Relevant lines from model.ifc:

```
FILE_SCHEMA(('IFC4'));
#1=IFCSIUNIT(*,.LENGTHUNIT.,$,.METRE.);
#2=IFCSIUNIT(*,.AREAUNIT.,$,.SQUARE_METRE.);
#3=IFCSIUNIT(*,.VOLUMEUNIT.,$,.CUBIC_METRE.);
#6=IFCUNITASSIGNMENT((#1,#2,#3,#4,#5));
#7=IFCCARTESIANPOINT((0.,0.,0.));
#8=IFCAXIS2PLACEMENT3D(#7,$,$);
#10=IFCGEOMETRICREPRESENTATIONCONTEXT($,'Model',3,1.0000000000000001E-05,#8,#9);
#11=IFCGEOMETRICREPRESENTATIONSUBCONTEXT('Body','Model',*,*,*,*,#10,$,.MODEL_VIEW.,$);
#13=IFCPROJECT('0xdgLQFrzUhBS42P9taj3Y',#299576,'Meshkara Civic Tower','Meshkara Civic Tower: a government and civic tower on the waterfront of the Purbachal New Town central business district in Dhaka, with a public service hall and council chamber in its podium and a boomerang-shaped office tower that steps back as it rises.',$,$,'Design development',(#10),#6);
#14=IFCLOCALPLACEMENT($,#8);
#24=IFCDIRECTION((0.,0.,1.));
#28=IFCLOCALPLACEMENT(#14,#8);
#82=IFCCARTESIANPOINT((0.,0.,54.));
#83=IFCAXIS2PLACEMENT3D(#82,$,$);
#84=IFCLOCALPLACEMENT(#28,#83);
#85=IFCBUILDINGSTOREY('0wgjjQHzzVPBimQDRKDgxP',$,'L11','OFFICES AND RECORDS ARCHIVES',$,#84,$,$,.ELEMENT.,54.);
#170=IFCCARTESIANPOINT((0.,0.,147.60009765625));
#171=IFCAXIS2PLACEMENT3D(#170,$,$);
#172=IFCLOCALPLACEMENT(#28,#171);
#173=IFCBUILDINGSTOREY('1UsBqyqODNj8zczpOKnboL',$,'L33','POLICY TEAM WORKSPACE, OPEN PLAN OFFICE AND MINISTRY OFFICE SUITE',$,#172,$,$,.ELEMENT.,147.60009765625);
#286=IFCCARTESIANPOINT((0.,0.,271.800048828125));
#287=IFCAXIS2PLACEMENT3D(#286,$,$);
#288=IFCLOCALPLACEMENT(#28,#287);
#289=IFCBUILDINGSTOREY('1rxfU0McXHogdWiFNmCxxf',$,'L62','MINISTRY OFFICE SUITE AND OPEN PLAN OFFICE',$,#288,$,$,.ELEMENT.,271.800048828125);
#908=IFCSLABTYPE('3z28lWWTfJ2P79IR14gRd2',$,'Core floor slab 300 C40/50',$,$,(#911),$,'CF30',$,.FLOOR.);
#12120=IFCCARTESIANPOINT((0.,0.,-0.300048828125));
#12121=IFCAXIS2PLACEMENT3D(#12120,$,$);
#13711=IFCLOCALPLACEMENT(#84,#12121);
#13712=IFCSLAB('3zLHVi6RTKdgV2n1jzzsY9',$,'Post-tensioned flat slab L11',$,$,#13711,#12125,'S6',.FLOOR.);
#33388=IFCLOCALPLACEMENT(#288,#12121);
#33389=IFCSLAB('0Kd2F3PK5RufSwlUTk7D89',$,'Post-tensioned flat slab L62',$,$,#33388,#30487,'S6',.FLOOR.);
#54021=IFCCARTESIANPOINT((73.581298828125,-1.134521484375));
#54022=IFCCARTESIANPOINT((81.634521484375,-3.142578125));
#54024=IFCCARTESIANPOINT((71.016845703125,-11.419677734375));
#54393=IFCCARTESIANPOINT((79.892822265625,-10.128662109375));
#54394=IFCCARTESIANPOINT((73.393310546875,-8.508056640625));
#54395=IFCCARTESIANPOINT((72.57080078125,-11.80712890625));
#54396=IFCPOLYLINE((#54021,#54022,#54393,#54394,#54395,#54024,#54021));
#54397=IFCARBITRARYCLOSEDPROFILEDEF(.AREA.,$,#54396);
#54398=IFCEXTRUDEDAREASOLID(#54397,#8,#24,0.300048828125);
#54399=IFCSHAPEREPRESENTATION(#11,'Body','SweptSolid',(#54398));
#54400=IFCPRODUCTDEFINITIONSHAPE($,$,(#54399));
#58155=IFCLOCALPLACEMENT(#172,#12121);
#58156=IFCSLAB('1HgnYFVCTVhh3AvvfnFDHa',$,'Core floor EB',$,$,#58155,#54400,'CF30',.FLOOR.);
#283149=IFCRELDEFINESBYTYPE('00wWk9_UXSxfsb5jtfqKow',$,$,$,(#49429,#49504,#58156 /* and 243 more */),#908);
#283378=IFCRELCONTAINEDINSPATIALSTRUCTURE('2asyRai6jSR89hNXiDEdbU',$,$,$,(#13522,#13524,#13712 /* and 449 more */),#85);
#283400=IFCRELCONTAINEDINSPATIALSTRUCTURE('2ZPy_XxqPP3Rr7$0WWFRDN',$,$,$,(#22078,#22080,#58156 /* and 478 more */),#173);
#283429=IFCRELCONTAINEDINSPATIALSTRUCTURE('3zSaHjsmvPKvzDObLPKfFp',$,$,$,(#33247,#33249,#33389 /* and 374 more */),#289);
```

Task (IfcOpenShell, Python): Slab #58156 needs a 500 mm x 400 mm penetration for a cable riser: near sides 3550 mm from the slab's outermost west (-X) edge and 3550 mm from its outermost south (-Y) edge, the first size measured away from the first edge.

```python
import numpy as np
import ifcopenshell
import ifcopenshell.api.feature
import ifcopenshell.api.geometry
import ifcopenshell.api.root
import ifcopenshell.geom
import ifcopenshell.util.placement
import ifcopenshell.util.representation
import ifcopenshell.util.shape
import ifcopenshell.util.unit

model = ifcopenshell.open("model.ifc")
unit_scale = ifcopenshell.util.unit.calculate_unit_scale(model)
settings = ifcopenshell.geom.settings()


def volume(element):
    """Net volume in cubic metres, openings subtracted."""
    shape = ifcopenshell.geom.create_shape(settings, element)
    return ifcopenshell.util.shape.get_volume(shape.geometry)


slab = model.by_guid("1HgnYFVCTVhh3AvvfnFDHa")
before = volume(slab)

# Extent in the slab's own axes, in metres. The edges named are its -X and -Y sides.
slab_shape = ifcopenshell.geom.create_shape(settings, slab)
vertices = ifcopenshell.util.shape.get_vertices(slab_shape.geometry)
x_min, y_min, bottom = vertices.min(axis=0)
top = vertices[:, 2].max()

opening = ifcopenshell.api.root.create_entity(model, ifc_class="IfcOpeningElement", name="Cable riser opening", predefined_type="OPENING")
context = ifcopenshell.util.representation.get_context(model, "Model", "Body", "MODEL_VIEW")
width, depth = 0.5, 0.4
outline = [(0.0, 0.0), (width, 0.0), (width, depth), (0.0, depth), (0.0, 0.0)]
# Overshoot both faces by 50 mm so the cut is clean.
shape = ifcopenshell.api.geometry.add_slab_representation(
    model, context=context, depth=top - bottom + 0.1, polyline=outline
)
ifcopenshell.api.geometry.assign_representation(model, product=opening, representation=shape)

matrix = ifcopenshell.util.placement.get_local_placement(slab.ObjectPlacement)
matrix[:, 3] = matrix @ np.append(np.array([x_min + 3.55, y_min + 3.55, bottom - 0.05]) / unit_scale, 1.0)
ifcopenshell.api.geometry.edit_object_placement(model, product=opening, matrix=matrix, is_si=False)
ifcopenshell.api.feature.add_feature(model, feature=opening, element=slab)

after = volume(slab)

print(f"slab volume {before:.3f} -> {after:.3f} m3")

model.write("model-out.ifc")
```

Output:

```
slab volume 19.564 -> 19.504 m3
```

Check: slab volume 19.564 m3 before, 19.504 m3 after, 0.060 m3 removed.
